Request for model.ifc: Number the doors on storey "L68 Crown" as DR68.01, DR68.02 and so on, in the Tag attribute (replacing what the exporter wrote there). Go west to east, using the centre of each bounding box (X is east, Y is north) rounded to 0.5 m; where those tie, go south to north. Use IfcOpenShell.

First a look at what the model holds.

```python
import ifcopenshell
import ifcopenshell.util.element
import ifcopenshell.util.placement

model = ifcopenshell.open("model.ifc")
print(model.schema)
storey = next(s for s in model.by_type("IfcBuildingStorey") if s.Name == "L68 Crown")
doors = [e for e in ifcopenshell.util.element.get_decomposition(storey) if e.is_a("IfcDoor")]
for e in sorted(doors, key=lambda e: e.id()):
    origin = ifcopenshell.util.placement.get_local_placement(e.ObjectPlacement)[:3, 3]
    print(e.id(), e.Tag, e.Name, origin.round(2) + 0.0, sep=" | ")
```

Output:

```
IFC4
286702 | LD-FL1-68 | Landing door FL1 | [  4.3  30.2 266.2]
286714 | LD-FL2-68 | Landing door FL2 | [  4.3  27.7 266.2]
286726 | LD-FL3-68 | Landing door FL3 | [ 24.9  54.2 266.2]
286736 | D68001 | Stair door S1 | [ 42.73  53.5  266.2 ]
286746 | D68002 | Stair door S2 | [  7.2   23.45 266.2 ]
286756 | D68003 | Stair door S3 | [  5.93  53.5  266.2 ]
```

```python
import ifcopenshell
import ifcopenshell.geom
import ifcopenshell.util.element
import ifcopenshell.util.shape

model = ifcopenshell.open("model.ifc")
settings = ifcopenshell.geom.settings()
settings.set("use-world-coords", True)


def centre(element):
    shape = ifcopenshell.geom.create_shape(settings, element)
    return ifcopenshell.util.shape.get_bbox_centroid(shape.geometry)


storey = next(s for s in model.by_type("IfcBuildingStorey") if s.Name == "L68 Crown")
doors = [e for e in ifcopenshell.util.element.get_decomposition(storey) if e.is_a("IfcDoor")]

# Insertion points can sit at a corner or the storey origin, so sort by the geometry (in metres).
centres = {e: centre(e) for e in doors}
doors.sort(key=lambda e: (round(centres[e][0] / 0.5), centres[e][1]))

for i, e in enumerate(doors, start=1):
    number = f"DR68.{i:02d}"
    e.Tag = number
    print(e.id(), number)

model.write("model_v2.ifc")
```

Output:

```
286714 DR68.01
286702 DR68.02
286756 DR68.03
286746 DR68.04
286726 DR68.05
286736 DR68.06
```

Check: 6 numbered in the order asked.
